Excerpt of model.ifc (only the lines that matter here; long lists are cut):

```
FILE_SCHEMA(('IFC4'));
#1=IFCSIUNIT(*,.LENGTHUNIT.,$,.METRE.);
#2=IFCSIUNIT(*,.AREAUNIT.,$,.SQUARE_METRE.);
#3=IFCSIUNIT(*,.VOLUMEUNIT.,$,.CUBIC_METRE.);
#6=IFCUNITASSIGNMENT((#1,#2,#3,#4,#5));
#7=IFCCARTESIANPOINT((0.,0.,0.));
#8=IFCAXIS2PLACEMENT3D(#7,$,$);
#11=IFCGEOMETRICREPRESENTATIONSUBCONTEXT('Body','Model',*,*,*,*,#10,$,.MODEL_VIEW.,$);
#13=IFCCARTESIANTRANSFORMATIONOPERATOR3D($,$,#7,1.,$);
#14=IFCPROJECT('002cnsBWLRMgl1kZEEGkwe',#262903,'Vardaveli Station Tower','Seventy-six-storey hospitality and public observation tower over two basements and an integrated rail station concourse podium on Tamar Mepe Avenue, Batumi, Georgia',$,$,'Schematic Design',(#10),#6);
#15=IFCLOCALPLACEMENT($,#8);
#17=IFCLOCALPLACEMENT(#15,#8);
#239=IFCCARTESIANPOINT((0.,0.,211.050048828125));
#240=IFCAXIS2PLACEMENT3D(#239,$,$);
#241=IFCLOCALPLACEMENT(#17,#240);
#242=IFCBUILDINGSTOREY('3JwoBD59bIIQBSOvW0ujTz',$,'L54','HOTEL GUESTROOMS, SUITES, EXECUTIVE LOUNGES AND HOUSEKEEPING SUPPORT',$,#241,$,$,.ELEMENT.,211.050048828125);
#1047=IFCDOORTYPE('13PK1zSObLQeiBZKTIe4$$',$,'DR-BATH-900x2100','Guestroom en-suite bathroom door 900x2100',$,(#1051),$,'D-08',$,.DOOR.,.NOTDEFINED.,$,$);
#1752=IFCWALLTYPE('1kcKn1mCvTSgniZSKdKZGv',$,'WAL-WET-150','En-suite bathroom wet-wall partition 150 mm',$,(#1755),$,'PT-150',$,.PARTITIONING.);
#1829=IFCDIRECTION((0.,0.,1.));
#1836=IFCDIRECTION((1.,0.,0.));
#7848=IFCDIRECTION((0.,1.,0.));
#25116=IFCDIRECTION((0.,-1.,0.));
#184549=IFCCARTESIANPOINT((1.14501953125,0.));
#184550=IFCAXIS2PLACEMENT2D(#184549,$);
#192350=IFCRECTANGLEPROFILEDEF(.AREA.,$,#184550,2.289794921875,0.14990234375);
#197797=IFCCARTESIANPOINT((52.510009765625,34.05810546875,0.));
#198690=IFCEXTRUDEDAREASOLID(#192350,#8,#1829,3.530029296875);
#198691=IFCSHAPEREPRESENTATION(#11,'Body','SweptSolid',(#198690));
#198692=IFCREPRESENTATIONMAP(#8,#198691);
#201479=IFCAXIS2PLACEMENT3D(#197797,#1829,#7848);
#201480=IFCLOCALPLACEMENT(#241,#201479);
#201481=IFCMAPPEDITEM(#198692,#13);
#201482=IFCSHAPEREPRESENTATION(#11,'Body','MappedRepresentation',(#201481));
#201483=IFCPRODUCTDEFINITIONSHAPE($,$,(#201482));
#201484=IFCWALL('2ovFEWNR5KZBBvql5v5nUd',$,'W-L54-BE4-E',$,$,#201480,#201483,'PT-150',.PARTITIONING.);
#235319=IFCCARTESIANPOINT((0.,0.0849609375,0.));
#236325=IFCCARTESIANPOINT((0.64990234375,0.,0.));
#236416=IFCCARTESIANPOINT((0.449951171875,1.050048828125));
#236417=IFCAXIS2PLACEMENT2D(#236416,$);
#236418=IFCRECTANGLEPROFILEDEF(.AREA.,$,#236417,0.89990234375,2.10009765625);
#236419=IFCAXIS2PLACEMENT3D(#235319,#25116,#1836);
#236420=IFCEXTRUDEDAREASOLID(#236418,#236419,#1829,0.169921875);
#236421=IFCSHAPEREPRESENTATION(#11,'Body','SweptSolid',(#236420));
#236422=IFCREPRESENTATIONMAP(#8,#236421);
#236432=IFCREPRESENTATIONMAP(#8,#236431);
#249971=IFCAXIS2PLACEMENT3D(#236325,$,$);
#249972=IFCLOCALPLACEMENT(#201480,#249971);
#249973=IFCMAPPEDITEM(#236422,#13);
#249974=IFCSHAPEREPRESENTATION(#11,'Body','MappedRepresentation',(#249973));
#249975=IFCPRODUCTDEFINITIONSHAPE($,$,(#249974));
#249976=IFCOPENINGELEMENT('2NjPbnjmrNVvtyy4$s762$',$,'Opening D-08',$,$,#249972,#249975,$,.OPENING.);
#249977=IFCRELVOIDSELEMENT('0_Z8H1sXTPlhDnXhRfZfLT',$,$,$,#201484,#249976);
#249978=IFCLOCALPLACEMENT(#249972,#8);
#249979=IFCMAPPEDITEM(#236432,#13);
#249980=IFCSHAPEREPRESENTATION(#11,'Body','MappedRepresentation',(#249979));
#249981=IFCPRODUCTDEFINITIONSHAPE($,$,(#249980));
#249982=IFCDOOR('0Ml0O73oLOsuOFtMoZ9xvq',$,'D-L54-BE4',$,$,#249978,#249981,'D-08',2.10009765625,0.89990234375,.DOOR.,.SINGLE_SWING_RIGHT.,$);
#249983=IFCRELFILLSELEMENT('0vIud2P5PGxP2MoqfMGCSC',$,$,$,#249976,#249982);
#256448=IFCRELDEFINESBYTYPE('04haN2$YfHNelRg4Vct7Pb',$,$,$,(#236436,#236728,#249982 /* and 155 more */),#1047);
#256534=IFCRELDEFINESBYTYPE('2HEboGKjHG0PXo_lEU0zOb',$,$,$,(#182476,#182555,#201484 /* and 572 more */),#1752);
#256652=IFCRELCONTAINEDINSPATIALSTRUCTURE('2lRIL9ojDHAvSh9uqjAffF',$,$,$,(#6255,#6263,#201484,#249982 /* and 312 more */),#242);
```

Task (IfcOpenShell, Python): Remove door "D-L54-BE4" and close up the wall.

```python
import ifcopenshell
import ifcopenshell.api.feature
import ifcopenshell.api.root
import ifcopenshell.geom
import ifcopenshell.util.shape

model = ifcopenshell.open("model.ifc")
settings = ifcopenshell.geom.settings()


def volume(element):
    """Net volume in cubic metres, openings subtracted."""
    shape = ifcopenshell.geom.create_shape(settings, element)
    return ifcopenshell.util.shape.get_volume(shape.geometry)


door = model.by_guid("0Ml0O73oLOsuOFtMoZ9xvq")
opening = door.FillsVoids[0].RelatingOpeningElement
wall = opening.VoidsElements[0].RelatingBuildingElement
before = volume(wall)

ifcopenshell.api.root.remove_product(model, product=door)
ifcopenshell.api.feature.remove_feature(model, feature=opening)

after = volume(wall)

print(f"wall volume {before:.3f} -> {after:.3f} m3")

model.write("model-out.ifc")
```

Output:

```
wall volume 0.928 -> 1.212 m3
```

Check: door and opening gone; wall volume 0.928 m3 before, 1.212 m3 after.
